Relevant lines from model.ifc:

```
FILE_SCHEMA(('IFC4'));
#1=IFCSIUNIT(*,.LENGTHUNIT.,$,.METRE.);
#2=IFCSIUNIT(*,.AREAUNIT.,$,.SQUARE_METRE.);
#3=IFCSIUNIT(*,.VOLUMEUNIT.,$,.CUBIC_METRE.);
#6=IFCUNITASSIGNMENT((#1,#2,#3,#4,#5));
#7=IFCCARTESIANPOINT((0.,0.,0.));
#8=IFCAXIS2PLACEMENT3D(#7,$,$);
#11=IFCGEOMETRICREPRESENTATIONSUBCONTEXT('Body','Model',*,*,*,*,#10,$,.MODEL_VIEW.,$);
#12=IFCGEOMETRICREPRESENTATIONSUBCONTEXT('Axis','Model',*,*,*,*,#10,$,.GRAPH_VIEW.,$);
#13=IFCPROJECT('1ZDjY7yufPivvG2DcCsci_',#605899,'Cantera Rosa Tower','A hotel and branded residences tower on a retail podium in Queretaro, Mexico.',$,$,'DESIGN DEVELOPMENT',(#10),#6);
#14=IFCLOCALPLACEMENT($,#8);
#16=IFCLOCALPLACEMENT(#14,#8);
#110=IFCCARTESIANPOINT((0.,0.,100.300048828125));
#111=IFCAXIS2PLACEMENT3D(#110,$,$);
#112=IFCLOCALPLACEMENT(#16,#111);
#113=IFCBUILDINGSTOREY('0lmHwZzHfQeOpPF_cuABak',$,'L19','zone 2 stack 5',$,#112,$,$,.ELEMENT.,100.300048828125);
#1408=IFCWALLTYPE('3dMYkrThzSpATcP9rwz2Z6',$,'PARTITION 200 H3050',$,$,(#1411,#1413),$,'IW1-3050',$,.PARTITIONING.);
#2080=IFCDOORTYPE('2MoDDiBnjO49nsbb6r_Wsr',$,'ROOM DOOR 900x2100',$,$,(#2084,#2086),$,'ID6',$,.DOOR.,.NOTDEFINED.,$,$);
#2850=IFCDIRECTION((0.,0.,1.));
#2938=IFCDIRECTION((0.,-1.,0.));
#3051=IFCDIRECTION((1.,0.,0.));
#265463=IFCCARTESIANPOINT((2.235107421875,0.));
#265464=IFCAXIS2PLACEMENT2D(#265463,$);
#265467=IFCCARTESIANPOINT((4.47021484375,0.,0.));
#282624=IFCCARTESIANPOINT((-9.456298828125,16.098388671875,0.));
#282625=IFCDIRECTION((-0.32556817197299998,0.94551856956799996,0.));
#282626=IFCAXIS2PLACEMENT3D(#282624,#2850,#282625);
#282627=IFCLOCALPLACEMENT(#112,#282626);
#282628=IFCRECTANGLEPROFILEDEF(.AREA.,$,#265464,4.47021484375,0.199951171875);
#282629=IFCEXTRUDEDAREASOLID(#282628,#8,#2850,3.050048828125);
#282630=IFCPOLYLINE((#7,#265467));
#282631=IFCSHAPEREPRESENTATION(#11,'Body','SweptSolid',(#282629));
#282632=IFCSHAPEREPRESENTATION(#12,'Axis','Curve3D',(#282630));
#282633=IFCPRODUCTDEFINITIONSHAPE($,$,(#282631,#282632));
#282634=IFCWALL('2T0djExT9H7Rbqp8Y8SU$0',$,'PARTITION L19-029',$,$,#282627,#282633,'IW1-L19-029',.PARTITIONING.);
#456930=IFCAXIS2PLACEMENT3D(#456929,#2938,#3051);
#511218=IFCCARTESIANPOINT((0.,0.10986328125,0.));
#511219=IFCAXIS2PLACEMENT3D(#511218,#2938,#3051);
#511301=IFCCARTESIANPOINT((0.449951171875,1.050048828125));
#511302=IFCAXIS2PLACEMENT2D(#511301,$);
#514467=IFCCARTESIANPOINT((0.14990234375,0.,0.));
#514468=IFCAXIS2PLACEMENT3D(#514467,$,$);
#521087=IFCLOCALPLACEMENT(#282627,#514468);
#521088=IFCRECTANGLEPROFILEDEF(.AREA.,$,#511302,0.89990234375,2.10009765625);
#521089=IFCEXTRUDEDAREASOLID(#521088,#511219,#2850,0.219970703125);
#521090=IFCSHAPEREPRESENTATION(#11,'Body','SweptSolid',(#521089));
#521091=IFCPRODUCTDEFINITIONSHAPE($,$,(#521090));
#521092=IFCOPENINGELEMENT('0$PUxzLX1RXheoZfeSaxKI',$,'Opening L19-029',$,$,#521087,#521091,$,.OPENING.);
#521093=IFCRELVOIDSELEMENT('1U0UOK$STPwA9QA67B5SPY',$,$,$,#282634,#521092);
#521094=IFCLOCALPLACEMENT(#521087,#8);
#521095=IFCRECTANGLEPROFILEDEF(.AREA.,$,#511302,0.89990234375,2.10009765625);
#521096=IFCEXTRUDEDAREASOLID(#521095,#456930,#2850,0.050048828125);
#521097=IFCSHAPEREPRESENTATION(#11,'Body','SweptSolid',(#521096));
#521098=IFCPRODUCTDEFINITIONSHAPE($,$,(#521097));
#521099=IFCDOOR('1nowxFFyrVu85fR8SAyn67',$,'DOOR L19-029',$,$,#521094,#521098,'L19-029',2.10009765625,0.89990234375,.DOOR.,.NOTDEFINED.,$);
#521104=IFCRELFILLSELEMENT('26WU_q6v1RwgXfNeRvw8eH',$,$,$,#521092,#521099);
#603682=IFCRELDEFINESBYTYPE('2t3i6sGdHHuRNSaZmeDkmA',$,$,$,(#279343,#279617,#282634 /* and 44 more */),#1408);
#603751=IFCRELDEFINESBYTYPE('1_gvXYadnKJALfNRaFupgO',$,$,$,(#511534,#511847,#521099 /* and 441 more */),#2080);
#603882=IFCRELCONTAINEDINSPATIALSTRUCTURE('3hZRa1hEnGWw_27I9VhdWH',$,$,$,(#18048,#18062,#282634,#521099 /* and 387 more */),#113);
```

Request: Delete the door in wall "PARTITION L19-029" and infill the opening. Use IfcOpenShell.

```python
import ifcopenshell
import ifcopenshell.api.feature
import ifcopenshell.api.root
import ifcopenshell.geom
import ifcopenshell.util.shape

model = ifcopenshell.open("model.ifc")
settings = ifcopenshell.geom.settings()


def volume(element):
    """Net volume in cubic metres, openings subtracted."""
    shape = ifcopenshell.geom.create_shape(settings, element)
    return ifcopenshell.util.shape.get_volume(shape.geometry)


door = model.by_guid("1nowxFFyrVu85fR8SAyn67")
opening = door.FillsVoids[0].RelatingOpeningElement
wall = opening.VoidsElements[0].RelatingBuildingElement
before = volume(wall)

ifcopenshell.api.root.remove_product(model, product=door)
ifcopenshell.api.feature.remove_feature(model, feature=opening)

after = volume(wall)

print(f"wall volume {before:.3f} -> {after:.3f} m3")

model.write("model_v2.ifc")
```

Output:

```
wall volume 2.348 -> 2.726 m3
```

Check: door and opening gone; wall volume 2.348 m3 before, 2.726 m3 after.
